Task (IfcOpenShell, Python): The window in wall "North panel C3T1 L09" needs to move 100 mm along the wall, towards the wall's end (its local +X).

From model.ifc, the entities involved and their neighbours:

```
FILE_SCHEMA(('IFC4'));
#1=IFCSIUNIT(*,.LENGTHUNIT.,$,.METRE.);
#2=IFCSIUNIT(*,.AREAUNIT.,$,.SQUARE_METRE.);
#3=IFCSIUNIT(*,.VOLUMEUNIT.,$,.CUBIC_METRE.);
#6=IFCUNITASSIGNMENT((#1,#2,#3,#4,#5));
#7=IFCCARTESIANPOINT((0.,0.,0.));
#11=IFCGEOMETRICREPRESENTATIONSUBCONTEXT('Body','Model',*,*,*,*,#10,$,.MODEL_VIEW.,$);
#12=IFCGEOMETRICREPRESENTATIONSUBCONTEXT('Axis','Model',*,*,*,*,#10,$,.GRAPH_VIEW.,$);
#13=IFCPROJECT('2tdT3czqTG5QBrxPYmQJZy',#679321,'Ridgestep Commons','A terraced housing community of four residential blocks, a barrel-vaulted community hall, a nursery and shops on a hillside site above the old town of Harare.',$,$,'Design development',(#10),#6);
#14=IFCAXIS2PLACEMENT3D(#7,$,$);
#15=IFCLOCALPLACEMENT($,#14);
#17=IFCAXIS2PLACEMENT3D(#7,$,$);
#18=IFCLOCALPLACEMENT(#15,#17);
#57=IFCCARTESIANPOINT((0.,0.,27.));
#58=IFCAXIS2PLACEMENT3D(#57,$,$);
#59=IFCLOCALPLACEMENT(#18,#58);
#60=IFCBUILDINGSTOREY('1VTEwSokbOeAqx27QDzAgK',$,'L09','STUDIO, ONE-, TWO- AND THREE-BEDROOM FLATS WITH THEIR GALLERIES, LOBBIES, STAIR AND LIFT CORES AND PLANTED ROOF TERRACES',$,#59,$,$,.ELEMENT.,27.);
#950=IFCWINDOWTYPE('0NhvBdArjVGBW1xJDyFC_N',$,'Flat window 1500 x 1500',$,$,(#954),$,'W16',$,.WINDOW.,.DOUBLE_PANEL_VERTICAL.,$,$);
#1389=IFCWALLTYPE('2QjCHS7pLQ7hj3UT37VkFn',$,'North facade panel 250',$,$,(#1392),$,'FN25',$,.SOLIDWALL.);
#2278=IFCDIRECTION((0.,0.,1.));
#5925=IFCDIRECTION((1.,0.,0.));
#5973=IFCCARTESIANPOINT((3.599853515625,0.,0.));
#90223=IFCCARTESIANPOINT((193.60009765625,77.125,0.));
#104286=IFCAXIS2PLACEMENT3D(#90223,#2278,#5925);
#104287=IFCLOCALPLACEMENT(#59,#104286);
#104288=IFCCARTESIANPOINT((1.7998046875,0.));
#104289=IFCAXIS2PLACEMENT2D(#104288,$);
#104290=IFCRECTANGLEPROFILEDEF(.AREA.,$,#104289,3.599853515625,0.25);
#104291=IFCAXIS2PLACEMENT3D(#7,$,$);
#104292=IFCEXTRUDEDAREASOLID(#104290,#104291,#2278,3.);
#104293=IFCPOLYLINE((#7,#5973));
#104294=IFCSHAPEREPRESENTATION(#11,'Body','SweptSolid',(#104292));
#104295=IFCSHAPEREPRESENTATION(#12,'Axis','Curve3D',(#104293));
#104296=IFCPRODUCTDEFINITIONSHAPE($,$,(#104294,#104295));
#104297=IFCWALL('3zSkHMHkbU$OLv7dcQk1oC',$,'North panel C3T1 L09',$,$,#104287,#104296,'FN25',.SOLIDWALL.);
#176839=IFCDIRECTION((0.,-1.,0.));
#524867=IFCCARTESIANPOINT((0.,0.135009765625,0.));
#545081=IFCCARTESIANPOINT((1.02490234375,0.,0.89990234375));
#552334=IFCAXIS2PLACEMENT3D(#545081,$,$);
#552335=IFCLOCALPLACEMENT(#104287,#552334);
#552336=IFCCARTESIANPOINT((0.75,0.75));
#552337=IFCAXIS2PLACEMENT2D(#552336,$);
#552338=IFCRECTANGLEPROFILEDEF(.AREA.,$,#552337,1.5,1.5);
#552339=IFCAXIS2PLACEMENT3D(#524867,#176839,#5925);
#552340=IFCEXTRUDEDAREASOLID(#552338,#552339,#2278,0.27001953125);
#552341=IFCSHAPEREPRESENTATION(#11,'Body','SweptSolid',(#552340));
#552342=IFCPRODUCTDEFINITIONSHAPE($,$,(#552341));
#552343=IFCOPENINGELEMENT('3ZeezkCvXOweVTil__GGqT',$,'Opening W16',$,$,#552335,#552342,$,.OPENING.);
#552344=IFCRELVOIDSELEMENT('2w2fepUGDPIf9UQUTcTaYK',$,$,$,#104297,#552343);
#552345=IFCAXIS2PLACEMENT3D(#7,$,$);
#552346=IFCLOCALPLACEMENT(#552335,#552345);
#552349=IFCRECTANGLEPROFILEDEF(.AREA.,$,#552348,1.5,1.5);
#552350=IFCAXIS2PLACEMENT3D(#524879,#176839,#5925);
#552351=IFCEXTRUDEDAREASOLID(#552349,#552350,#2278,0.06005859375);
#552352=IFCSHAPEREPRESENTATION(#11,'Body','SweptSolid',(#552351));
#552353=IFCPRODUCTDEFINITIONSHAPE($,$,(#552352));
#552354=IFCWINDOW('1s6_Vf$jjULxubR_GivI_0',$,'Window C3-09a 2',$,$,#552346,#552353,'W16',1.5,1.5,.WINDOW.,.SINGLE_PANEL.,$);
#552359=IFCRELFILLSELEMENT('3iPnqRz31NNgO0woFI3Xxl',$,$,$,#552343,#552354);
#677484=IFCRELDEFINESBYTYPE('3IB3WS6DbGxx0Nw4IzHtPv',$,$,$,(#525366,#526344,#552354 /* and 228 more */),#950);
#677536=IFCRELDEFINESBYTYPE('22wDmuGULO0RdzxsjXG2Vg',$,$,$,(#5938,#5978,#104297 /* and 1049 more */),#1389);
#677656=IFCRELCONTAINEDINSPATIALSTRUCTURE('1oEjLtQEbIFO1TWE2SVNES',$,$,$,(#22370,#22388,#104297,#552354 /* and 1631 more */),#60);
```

```python
import ifcopenshell
import ifcopenshell.api.geometry
import ifcopenshell.util.placement

model = ifcopenshell.open("model.ifc")

window = model.by_guid("1s6_Vf$jjULxubR_GivI_0")
opening = window.FillsVoids[0].RelatingOpeningElement
wall = opening.VoidsElements[0].RelatingBuildingElement

wall_matrix = ifcopenshell.util.placement.get_local_placement(wall.ObjectPlacement)
shift = wall_matrix[:3, 0] * 0.1
before = ifcopenshell.util.placement.get_local_placement(window.ObjectPlacement)[:3, 3].copy()

# The window is placed relative to its opening, so it follows when the opening moves.
matrix = ifcopenshell.util.placement.get_local_placement(opening.ObjectPlacement)
matrix[:3, 3] += shift
ifcopenshell.api.geometry.edit_object_placement(
    model, product=opening, matrix=matrix, is_si=False, should_transform_children=True
)

after = ifcopenshell.util.placement.get_local_placement(window.ObjectPlacement)[:3, 3]
print("window moved by", (after - before).round(3) + 0.0)

model.write("model_v2.ifc")
```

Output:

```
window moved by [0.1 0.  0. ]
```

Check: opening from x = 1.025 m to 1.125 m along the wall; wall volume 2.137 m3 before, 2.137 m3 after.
